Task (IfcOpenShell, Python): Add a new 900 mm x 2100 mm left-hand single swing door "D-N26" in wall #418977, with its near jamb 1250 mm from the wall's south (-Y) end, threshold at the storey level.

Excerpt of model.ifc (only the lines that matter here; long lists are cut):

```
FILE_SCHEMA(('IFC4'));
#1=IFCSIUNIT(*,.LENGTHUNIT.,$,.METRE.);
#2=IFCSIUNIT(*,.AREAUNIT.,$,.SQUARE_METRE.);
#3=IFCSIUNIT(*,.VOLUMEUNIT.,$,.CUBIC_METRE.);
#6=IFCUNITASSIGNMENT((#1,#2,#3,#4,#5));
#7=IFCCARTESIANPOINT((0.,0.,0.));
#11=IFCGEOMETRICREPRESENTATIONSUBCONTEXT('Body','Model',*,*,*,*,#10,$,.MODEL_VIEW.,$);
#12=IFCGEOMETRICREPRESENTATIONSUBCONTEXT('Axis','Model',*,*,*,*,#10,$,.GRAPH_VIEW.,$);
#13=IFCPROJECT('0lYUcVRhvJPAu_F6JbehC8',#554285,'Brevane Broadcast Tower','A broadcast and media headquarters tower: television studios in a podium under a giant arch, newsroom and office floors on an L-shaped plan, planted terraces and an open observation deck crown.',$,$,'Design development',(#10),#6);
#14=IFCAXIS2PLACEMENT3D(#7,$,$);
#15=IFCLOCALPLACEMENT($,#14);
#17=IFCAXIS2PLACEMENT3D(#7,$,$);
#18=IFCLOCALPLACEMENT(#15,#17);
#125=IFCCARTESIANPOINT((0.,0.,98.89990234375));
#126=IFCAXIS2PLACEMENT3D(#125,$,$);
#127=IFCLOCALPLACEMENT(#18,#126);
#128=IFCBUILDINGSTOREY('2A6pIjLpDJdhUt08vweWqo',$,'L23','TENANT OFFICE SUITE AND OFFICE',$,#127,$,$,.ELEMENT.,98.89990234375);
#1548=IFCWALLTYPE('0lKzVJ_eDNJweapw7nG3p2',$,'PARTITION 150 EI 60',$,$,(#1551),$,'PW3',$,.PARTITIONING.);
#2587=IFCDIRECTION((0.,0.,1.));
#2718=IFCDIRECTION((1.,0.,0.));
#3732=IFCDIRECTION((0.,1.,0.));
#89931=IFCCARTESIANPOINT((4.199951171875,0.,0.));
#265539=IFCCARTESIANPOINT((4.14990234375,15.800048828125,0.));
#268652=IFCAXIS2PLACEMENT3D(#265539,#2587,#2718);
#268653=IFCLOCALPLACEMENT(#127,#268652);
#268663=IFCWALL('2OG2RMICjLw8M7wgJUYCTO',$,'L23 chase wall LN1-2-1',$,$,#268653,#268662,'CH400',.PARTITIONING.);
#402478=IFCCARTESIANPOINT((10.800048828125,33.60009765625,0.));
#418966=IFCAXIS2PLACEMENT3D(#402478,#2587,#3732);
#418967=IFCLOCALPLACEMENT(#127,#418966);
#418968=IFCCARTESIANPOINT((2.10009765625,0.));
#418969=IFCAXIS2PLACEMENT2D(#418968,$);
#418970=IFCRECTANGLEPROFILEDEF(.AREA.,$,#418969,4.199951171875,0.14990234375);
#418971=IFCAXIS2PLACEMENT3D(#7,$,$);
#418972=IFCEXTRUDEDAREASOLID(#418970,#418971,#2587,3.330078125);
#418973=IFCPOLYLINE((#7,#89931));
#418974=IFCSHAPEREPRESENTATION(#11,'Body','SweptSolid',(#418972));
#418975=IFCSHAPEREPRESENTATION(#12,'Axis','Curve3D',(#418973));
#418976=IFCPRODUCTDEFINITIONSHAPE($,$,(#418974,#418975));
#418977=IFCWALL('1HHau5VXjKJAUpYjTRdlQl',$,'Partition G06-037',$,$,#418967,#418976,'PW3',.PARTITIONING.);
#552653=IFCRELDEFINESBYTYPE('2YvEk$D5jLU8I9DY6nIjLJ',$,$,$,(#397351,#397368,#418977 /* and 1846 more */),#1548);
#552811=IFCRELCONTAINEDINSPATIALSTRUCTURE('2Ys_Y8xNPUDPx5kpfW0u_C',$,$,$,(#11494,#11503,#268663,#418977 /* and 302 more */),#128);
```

```python
import numpy as np
import ifcopenshell
import ifcopenshell.api.feature
import ifcopenshell.api.geometry
import ifcopenshell.api.root
import ifcopenshell.api.spatial
import ifcopenshell.geom
import ifcopenshell.util.element
import ifcopenshell.util.placement
import ifcopenshell.util.representation
import ifcopenshell.util.shape
import ifcopenshell.util.unit

model = ifcopenshell.open("model.ifc")
unit_scale = ifcopenshell.util.unit.calculate_unit_scale(model)
settings = ifcopenshell.geom.settings()


def volume(element):
    """Net volume in cubic metres, openings subtracted."""
    shape = ifcopenshell.geom.create_shape(settings, element)
    return ifcopenshell.util.shape.get_volume(shape.geometry)


wall = model.by_guid("1HHau5VXjKJAUpYjTRdlQl")
storey = ifcopenshell.util.element.get_container(wall, ifc_class="IfcBuildingStorey")
context = ifcopenshell.util.representation.get_context(model, "Model", "Body", "MODEL_VIEW")
before = volume(wall)

width, height, from_end, sill = 0.9, 2.1, 1.25, 0.0  # metres

# The wall runs along its own X axis, and the end named is its -X end.
wall_shape = ifcopenshell.geom.create_shape(settings, wall)
x, y, z = ifcopenshell.util.shape.get_vertices(wall_shape.geometry).T
start = x.min() + from_end
face, thickness = float(y.min()), float(y.max() - y.min())
wall_matrix = ifcopenshell.util.placement.get_local_placement(wall.ObjectPlacement)
level = ifcopenshell.util.placement.get_local_placement(storey.ObjectPlacement)[2, 3]


def in_wall(x, y):
    """Placement at x, y metres in the wall's axes, at sill height."""
    matrix = wall_matrix.copy()
    matrix[:, 3] = wall_matrix @ np.array([x / unit_scale, y / unit_scale, 0.0, 1.0])
    matrix[2, 3] = level + sill / unit_scale
    return matrix


# Opening: a box that overshoots both wall faces by 50 mm.
opening = ifcopenshell.api.root.create_entity(model, ifc_class="IfcOpeningElement", predefined_type="OPENING")
box = ifcopenshell.api.geometry.add_wall_representation(
    model, context=context, length=width, height=height, thickness=thickness + 0.1
)
ifcopenshell.api.geometry.assign_representation(model, product=opening, representation=box)
ifcopenshell.api.geometry.edit_object_placement(model, product=opening, matrix=in_wall(start, face - 0.05), is_si=False)
ifcopenshell.api.feature.add_feature(model, feature=opening, element=wall)

door = ifcopenshell.api.root.create_entity(model, ifc_class="IfcDoor", name="D-N26", predefined_type="DOOR")
door.OverallWidth, door.OverallHeight = width / unit_scale, height / unit_scale
door.OperationType = "SINGLE_SWING_LEFT"
body = ifcopenshell.api.geometry.add_door_representation(
    model,
    context=context,
    overall_width=door.OverallWidth,
    overall_height=door.OverallHeight,
    operation_type="SINGLE_SWING_LEFT",
    lining_properties={"LiningDepth": thickness / unit_scale, "ThresholdDepth": thickness / unit_scale},
)
ifcopenshell.api.geometry.assign_representation(model, product=door, representation=body)
ifcopenshell.api.spatial.assign_container(model, products=[door], relating_structure=storey)
ifcopenshell.api.feature.add_filling(model, opening=opening, element=door)

# The lining spans the wall, so the door starts at the wall face.
ifcopenshell.api.geometry.edit_object_placement(model, product=door, matrix=in_wall(start, face), is_si=False)

after = volume(wall)

print(f"wall volume {before:.3f} -> {after:.3f} m3")

model.write("model_updated.ifc")
```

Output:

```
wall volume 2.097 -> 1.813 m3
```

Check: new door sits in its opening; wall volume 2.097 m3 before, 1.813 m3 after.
